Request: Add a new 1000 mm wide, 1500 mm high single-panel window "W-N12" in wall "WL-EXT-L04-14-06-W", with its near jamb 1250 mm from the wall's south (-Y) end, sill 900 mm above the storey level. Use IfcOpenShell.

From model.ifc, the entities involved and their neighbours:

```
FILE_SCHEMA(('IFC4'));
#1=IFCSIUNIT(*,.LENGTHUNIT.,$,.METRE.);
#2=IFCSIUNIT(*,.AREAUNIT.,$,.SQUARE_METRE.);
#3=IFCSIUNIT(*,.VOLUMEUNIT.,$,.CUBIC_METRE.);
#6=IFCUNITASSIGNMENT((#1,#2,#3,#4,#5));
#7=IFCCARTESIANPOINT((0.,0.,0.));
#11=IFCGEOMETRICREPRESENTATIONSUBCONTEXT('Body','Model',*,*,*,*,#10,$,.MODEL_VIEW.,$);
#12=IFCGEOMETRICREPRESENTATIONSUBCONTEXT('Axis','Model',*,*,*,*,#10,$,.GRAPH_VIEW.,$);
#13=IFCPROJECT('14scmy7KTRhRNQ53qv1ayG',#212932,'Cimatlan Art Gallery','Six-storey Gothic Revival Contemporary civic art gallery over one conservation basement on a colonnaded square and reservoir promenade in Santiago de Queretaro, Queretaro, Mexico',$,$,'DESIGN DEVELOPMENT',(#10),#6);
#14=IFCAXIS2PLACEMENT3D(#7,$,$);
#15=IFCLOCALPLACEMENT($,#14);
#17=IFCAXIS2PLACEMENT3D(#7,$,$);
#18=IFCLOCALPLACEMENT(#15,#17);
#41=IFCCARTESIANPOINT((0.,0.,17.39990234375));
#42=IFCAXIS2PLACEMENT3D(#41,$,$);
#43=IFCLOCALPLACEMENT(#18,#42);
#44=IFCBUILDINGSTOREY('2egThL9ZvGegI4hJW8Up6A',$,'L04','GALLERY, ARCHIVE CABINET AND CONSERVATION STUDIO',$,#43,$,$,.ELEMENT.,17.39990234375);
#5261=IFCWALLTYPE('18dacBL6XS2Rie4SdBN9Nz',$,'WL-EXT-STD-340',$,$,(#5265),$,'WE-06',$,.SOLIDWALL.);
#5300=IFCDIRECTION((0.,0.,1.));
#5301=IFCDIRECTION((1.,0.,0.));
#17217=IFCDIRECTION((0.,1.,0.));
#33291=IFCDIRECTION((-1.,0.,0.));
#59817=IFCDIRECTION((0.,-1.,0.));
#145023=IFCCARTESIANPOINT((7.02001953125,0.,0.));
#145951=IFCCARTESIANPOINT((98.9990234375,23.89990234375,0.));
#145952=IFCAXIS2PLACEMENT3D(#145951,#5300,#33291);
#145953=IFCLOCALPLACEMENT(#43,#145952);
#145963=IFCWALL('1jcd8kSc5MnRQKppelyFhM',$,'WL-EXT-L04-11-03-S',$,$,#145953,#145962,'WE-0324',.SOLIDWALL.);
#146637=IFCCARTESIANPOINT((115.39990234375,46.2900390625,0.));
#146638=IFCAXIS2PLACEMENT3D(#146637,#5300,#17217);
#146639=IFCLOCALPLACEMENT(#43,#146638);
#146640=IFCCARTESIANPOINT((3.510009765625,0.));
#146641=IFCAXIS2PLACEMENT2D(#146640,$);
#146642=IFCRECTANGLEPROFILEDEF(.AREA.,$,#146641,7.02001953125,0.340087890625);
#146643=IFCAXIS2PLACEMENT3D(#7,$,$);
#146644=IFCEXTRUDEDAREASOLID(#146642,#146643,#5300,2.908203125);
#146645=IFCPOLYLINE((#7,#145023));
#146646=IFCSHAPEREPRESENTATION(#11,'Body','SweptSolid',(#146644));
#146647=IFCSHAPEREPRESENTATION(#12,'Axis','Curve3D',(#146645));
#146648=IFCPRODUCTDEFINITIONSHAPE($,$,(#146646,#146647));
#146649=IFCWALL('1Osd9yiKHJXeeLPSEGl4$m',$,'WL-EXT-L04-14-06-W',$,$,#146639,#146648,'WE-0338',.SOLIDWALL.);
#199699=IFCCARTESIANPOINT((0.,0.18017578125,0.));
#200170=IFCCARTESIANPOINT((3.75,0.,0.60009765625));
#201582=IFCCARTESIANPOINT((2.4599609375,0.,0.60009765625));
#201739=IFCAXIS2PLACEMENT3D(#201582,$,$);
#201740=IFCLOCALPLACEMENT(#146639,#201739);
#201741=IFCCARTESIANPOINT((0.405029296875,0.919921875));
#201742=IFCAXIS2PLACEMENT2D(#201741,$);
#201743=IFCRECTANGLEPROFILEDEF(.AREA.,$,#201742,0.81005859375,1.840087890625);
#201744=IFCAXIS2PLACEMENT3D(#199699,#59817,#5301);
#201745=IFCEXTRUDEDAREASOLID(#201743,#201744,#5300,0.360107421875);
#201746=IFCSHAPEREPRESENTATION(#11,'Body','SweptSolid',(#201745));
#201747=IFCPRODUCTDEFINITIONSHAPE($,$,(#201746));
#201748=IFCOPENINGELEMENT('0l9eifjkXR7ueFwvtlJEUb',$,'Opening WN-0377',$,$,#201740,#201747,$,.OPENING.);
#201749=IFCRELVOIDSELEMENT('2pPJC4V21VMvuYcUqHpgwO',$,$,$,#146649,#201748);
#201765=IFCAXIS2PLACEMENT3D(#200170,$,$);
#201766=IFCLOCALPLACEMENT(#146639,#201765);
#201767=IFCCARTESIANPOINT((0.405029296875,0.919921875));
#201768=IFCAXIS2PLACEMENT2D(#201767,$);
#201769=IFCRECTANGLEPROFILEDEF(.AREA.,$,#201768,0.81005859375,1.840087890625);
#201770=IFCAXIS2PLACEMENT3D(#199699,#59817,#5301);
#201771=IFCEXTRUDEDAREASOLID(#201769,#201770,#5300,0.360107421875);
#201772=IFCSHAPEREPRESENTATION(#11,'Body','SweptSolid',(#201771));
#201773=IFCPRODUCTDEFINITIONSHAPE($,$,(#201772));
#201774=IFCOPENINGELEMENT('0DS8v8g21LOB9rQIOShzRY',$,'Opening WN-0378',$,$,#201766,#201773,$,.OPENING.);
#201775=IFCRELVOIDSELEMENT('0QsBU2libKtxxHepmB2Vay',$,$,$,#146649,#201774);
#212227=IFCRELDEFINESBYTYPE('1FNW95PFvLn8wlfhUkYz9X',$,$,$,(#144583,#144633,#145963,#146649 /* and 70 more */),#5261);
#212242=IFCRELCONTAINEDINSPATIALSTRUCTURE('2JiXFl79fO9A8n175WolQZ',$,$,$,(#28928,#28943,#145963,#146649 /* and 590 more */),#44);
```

```python
import numpy as np
import ifcopenshell
import ifcopenshell.api.feature
import ifcopenshell.api.geometry
import ifcopenshell.api.root
import ifcopenshell.api.spatial
import ifcopenshell.geom
import ifcopenshell.util.element
import ifcopenshell.util.placement
import ifcopenshell.util.representation
import ifcopenshell.util.shape
import ifcopenshell.util.unit

model = ifcopenshell.open("model.ifc")
unit_scale = ifcopenshell.util.unit.calculate_unit_scale(model)
settings = ifcopenshell.geom.settings()


def volume(element):
    """Net volume in cubic metres, openings subtracted."""
    shape = ifcopenshell.geom.create_shape(settings, element)
    return ifcopenshell.util.shape.get_volume(shape.geometry)


wall = model.by_guid("1Osd9yiKHJXeeLPSEGl4$m")
storey = ifcopenshell.util.element.get_container(wall, ifc_class="IfcBuildingStorey")
context = ifcopenshell.util.representation.get_context(model, "Model", "Body", "MODEL_VIEW")
before = volume(wall)

width, height, from_end, sill = 1, 1.5, 1.25, 0.9  # metres

# The wall runs along its own X axis, and the end named is its -X end.
wall_shape = ifcopenshell.geom.create_shape(settings, wall)
x, y, z = ifcopenshell.util.shape.get_vertices(wall_shape.geometry).T
start = x.min() + from_end
face, thickness = float(y.min()), float(y.max() - y.min())
wall_matrix = ifcopenshell.util.placement.get_local_placement(wall.ObjectPlacement)
level = ifcopenshell.util.placement.get_local_placement(storey.ObjectPlacement)[2, 3]


def in_wall(x, y):
    """Placement at x, y metres in the wall's axes, at sill height."""
    matrix = wall_matrix.copy()
    matrix[:, 3] = wall_matrix @ np.array([x / unit_scale, y / unit_scale, 0.0, 1.0])
    matrix[2, 3] = level + sill / unit_scale
    return matrix


# Opening: a box that overshoots both wall faces by 50 mm.
opening = ifcopenshell.api.root.create_entity(model, ifc_class="IfcOpeningElement", predefined_type="OPENING")
box = ifcopenshell.api.geometry.add_wall_representation(
    model, context=context, length=width, height=height, thickness=thickness + 0.1
)
ifcopenshell.api.geometry.assign_representation(model, product=opening, representation=box)
ifcopenshell.api.geometry.edit_object_placement(model, product=opening, matrix=in_wall(start, face - 0.05), is_si=False)
ifcopenshell.api.feature.add_feature(model, feature=opening, element=wall)

window = ifcopenshell.api.root.create_entity(model, ifc_class="IfcWindow", name="W-N12", predefined_type="WINDOW")
window.OverallWidth, window.OverallHeight = width / unit_scale, height / unit_scale
window.PartitioningType = "SINGLE_PANEL"
body = ifcopenshell.api.geometry.add_window_representation(
    model,
    context=context,
    overall_width=window.OverallWidth,
    overall_height=window.OverallHeight,
    partition_type="SINGLE_PANEL",
)
ifcopenshell.api.geometry.assign_representation(model, product=window, representation=body)
ifcopenshell.api.spatial.assign_container(model, products=[window], relating_structure=storey)
ifcopenshell.api.feature.add_filling(model, opening=opening, element=window)

# Centre the window in the wall's thickness.
ifcopenshell.api.geometry.edit_object_placement(model, product=window, matrix=in_wall(start, face), is_si=False)
window_shape = ifcopenshell.geom.create_shape(settings, window)
depth = ifcopenshell.util.shape.get_vertices(window_shape.geometry)[:, 1]
offset = face + thickness / 2 - (depth.min() + depth.max()) / 2
ifcopenshell.api.geometry.edit_object_placement(model, product=window, matrix=in_wall(start, offset), is_si=False)

after = volume(wall)

print(f"wall volume {before:.3f} -> {after:.3f} m3")

model.write("model_edited.ifc")
```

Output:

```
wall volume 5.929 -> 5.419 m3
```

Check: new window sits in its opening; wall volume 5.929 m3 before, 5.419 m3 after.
